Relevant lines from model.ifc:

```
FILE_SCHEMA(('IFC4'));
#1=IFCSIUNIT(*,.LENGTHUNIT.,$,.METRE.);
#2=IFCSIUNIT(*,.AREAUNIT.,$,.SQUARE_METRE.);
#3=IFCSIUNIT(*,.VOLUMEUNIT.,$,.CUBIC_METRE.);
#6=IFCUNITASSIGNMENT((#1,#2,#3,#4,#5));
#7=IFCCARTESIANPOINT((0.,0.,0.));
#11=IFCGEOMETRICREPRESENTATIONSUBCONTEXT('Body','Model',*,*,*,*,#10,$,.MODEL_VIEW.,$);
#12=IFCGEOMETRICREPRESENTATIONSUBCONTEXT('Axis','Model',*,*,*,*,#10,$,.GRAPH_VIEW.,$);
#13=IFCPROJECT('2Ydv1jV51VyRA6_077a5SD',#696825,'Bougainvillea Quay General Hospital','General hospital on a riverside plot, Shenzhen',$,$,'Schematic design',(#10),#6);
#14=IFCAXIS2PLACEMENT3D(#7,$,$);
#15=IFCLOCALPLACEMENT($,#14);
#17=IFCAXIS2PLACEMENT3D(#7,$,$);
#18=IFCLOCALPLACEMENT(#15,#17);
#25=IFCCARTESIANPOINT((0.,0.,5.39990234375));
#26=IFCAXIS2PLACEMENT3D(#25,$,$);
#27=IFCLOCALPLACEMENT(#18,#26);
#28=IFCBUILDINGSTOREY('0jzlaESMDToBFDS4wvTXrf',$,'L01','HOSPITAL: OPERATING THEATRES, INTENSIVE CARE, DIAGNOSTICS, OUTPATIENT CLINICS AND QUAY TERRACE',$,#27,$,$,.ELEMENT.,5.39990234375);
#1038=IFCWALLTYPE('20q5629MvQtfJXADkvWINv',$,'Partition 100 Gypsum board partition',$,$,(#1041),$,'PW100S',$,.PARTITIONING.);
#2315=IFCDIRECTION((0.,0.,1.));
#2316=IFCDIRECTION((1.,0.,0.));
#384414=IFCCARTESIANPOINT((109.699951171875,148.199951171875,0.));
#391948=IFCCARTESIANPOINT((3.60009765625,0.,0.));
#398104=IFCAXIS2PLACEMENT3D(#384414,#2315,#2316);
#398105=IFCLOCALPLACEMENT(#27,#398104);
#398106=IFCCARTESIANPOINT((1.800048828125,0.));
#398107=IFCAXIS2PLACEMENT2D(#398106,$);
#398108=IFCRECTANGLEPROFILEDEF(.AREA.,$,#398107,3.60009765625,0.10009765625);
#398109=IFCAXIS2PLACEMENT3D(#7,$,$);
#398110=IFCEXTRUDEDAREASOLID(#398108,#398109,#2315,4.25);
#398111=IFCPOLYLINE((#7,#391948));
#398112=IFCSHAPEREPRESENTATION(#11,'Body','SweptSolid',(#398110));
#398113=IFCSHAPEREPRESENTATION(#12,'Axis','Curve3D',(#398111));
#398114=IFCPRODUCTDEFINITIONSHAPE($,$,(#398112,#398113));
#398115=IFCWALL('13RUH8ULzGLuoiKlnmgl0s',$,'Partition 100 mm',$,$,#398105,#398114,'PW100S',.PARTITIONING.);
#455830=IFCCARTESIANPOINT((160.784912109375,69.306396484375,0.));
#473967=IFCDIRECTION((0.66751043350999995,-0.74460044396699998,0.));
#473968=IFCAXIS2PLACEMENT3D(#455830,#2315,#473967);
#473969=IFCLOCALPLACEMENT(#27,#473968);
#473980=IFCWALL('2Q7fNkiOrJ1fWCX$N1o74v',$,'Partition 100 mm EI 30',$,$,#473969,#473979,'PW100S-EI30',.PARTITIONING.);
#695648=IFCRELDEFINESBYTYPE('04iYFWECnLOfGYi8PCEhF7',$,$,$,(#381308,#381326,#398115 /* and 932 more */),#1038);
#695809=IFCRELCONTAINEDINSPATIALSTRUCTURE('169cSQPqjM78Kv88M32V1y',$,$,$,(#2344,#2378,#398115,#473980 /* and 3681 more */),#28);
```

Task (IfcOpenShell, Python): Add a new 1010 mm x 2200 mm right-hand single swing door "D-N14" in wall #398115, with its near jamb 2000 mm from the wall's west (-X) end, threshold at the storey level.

```python
import numpy as np
import ifcopenshell
import ifcopenshell.api.feature
import ifcopenshell.api.geometry
import ifcopenshell.api.root
import ifcopenshell.api.spatial
import ifcopenshell.geom
import ifcopenshell.util.element
import ifcopenshell.util.placement
import ifcopenshell.util.representation
import ifcopenshell.util.shape
import ifcopenshell.util.unit

model = ifcopenshell.open("model.ifc")
unit_scale = ifcopenshell.util.unit.calculate_unit_scale(model)
settings = ifcopenshell.geom.settings()


def volume(element):
    """Net volume in cubic metres, openings subtracted."""
    shape = ifcopenshell.geom.create_shape(settings, element)
    return ifcopenshell.util.shape.get_volume(shape.geometry)


wall = model.by_guid("13RUH8ULzGLuoiKlnmgl0s")
storey = ifcopenshell.util.element.get_container(wall, ifc_class="IfcBuildingStorey")
context = ifcopenshell.util.representation.get_context(model, "Model", "Body", "MODEL_VIEW")
before = volume(wall)

width, height, from_end, sill = 1.01, 2.2, 2, 0.0  # metres

# The wall runs along its own X axis, and the end named is its -X end.
wall_shape = ifcopenshell.geom.create_shape(settings, wall)
x, y, z = ifcopenshell.util.shape.get_vertices(wall_shape.geometry).T
start = x.min() + from_end
face, thickness = float(y.min()), float(y.max() - y.min())
wall_matrix = ifcopenshell.util.placement.get_local_placement(wall.ObjectPlacement)
level = ifcopenshell.util.placement.get_local_placement(storey.ObjectPlacement)[2, 3]


def in_wall(x, y):
    """Placement at x, y metres in the wall's axes, at sill height."""
    matrix = wall_matrix.copy()
    matrix[:, 3] = wall_matrix @ np.array([x / unit_scale, y / unit_scale, 0.0, 1.0])
    matrix[2, 3] = level + sill / unit_scale
    return matrix


# Opening: a box that overshoots both wall faces by 50 mm.
opening = ifcopenshell.api.root.create_entity(model, ifc_class="IfcOpeningElement", predefined_type="OPENING")
box = ifcopenshell.api.geometry.add_wall_representation(
    model, context=context, length=width, height=height, thickness=thickness + 0.1
)
ifcopenshell.api.geometry.assign_representation(model, product=opening, representation=box)
ifcopenshell.api.geometry.edit_object_placement(model, product=opening, matrix=in_wall(start, face - 0.05), is_si=False)
ifcopenshell.api.feature.add_feature(model, feature=opening, element=wall)

door = ifcopenshell.api.root.create_entity(model, ifc_class="IfcDoor", name="D-N14", predefined_type="DOOR")
door.OverallWidth, door.OverallHeight = width / unit_scale, height / unit_scale
door.OperationType = "SINGLE_SWING_RIGHT"
body = ifcopenshell.api.geometry.add_door_representation(
    model,
    context=context,
    overall_width=door.OverallWidth,
    overall_height=door.OverallHeight,
    operation_type="SINGLE_SWING_RIGHT",
    lining_properties={"LiningDepth": thickness / unit_scale, "ThresholdDepth": thickness / unit_scale},
)
ifcopenshell.api.geometry.assign_representation(model, product=door, representation=body)
ifcopenshell.api.spatial.assign_container(model, products=[door], relating_structure=storey)
ifcopenshell.api.feature.add_filling(model, opening=opening, element=door)

# The lining spans the wall, so the door starts at the wall face.
ifcopenshell.api.geometry.edit_object_placement(model, product=door, matrix=in_wall(start, face), is_si=False)

after = volume(wall)

print(f"wall volume {before:.3f} -> {after:.3f} m3")

model.write("model_updated.ifc")
```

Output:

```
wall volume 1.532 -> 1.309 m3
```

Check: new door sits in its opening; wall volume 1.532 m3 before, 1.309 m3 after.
